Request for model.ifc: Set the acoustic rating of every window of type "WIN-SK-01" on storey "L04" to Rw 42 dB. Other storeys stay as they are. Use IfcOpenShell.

First a look at what the model holds.

```python
import ifcopenshell
import ifcopenshell.util.element

model = ifcopenshell.open("model.ifc")
print(model.schema)
storey = next(s for s in model.by_type("IfcBuildingStorey") if s.Name == "L04")
windows = [e for e in ifcopenshell.util.element.get_decomposition(storey) if e.is_a("IfcWindow")]
seen = {}
for e in windows:
    element_type = ifcopenshell.util.element.get_type(e)
    key = (element_type.Name if element_type != e and element_type else None, ifcopenshell.util.element.get_pset(e, "Pset_WindowCommon", "AcousticRating"))
    seen[key] = seen.get(key, 0) + 1
for (name, value), count in sorted(seen.items(), key=str):
    print(count, "x", name, "|", value)
```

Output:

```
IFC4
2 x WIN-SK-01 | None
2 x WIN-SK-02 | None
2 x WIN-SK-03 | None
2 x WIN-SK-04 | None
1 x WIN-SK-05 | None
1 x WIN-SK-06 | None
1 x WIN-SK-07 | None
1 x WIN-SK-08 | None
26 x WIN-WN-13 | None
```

```python
import ifcopenshell
import ifcopenshell.api.pset
import ifcopenshell.util.element

model = ifcopenshell.open("model.ifc")

storey = next(s for s in model.by_type("IfcBuildingStorey") if s.Name == "L04")
windows = [e for e in ifcopenshell.util.element.get_decomposition(storey) if e.is_a("IfcWindow")]

count = 0
for e in windows:
    element_type = ifcopenshell.util.element.get_type(e)
    if element_type in (None, e) or element_type.Name != "WIN-SK-01":
        continue
    # add_pset returns the element's existing set when there is one.
    pset = ifcopenshell.api.pset.add_pset(model, product=e, name="Pset_WindowCommon")
    ifcopenshell.api.pset.edit_pset(model, pset=pset, properties={"AcousticRating": "Rw 42 dB"})
    count += 1

print(count, "windows updated")

model.write("model_rev.ifc")
```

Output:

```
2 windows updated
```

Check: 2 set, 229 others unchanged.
